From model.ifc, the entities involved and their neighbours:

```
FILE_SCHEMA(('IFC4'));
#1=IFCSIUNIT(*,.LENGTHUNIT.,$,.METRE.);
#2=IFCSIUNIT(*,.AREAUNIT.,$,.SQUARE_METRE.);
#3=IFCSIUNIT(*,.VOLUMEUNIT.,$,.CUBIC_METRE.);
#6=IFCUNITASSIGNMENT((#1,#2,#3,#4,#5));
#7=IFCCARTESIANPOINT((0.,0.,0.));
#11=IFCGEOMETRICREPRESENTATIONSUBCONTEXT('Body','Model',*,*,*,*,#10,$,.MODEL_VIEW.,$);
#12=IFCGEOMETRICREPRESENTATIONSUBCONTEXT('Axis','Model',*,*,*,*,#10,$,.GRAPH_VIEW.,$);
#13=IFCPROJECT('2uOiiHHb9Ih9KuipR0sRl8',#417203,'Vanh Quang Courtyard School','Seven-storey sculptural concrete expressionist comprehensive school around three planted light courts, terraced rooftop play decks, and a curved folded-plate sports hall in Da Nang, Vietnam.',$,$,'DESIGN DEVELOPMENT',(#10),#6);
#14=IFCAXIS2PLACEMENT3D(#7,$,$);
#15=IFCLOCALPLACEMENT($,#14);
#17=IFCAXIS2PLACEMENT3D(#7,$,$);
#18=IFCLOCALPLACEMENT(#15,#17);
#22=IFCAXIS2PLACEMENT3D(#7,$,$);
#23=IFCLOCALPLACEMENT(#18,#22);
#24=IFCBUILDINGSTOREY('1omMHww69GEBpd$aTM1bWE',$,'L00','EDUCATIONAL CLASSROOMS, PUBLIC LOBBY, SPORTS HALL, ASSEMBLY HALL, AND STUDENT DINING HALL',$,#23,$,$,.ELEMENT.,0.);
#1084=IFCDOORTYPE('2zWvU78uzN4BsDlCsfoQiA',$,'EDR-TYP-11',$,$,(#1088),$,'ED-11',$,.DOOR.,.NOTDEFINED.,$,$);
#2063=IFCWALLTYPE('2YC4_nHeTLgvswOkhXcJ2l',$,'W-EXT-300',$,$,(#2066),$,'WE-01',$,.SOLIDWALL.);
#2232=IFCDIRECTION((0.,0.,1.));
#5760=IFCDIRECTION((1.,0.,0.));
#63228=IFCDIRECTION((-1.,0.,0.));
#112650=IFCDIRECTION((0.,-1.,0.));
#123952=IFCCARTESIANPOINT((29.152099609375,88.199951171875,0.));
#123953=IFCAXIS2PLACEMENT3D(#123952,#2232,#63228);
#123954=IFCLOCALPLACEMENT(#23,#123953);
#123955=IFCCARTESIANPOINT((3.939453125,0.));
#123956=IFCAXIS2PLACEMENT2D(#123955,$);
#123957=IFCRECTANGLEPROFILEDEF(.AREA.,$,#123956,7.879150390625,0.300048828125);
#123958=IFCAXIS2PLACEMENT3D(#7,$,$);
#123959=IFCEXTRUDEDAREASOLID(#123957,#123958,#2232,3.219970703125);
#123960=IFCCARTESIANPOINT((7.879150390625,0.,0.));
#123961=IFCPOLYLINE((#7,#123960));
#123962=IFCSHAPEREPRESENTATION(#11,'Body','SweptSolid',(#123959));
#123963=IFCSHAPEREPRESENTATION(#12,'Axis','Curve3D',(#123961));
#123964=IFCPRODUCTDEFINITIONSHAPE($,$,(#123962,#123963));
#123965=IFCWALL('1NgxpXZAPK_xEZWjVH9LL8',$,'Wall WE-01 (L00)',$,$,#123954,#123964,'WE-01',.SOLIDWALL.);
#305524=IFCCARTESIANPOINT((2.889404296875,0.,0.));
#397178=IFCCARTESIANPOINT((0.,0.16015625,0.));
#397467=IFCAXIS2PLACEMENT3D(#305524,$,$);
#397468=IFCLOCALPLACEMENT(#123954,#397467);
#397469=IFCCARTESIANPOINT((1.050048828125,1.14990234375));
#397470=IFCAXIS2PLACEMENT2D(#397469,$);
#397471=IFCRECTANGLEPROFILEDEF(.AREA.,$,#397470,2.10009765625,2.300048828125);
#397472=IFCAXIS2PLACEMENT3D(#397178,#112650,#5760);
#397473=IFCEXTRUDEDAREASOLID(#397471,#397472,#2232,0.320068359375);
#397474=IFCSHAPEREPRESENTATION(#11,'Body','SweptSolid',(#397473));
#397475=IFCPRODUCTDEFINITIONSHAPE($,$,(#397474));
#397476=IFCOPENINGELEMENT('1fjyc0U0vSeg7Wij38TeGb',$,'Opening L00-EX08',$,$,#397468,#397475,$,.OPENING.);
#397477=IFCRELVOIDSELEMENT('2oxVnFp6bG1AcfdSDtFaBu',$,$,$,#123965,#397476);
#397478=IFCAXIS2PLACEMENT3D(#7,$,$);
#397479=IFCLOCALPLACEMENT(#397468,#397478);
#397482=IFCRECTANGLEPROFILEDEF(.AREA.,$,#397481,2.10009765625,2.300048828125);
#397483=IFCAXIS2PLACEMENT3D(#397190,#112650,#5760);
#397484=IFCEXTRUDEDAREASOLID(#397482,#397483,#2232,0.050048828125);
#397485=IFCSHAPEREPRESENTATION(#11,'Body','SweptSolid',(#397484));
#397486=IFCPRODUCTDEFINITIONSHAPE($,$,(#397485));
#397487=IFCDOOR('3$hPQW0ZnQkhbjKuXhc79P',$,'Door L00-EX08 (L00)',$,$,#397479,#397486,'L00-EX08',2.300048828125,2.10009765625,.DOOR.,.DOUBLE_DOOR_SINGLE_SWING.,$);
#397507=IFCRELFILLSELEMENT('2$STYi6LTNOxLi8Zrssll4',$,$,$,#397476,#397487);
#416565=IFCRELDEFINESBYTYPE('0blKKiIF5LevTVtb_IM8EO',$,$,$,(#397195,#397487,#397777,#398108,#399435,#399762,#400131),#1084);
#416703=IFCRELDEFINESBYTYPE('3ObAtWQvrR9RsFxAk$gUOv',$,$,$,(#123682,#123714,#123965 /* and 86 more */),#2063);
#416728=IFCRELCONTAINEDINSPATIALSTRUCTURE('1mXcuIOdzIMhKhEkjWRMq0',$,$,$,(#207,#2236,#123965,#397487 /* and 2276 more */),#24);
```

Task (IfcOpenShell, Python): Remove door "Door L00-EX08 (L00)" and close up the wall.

```python
import ifcopenshell
import ifcopenshell.api.feature
import ifcopenshell.api.root
import ifcopenshell.geom
import ifcopenshell.util.shape

model = ifcopenshell.open("model.ifc")
settings = ifcopenshell.geom.settings()


def volume(element):
    """Net volume in cubic metres, openings subtracted."""
    shape = ifcopenshell.geom.create_shape(settings, element)
    return ifcopenshell.util.shape.get_volume(shape.geometry)


door = model.by_guid("3$hPQW0ZnQkhbjKuXhc79P")
opening = door.FillsVoids[0].RelatingOpeningElement
wall = opening.VoidsElements[0].RelatingBuildingElement
before = volume(wall)

ifcopenshell.api.root.remove_product(model, product=door)
ifcopenshell.api.feature.remove_feature(model, feature=opening)

after = volume(wall)

print(f"wall volume {before:.3f} -> {after:.3f} m3")

model.write("model_rev.ifc")
```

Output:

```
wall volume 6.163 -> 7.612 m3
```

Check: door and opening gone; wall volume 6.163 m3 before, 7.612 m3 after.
